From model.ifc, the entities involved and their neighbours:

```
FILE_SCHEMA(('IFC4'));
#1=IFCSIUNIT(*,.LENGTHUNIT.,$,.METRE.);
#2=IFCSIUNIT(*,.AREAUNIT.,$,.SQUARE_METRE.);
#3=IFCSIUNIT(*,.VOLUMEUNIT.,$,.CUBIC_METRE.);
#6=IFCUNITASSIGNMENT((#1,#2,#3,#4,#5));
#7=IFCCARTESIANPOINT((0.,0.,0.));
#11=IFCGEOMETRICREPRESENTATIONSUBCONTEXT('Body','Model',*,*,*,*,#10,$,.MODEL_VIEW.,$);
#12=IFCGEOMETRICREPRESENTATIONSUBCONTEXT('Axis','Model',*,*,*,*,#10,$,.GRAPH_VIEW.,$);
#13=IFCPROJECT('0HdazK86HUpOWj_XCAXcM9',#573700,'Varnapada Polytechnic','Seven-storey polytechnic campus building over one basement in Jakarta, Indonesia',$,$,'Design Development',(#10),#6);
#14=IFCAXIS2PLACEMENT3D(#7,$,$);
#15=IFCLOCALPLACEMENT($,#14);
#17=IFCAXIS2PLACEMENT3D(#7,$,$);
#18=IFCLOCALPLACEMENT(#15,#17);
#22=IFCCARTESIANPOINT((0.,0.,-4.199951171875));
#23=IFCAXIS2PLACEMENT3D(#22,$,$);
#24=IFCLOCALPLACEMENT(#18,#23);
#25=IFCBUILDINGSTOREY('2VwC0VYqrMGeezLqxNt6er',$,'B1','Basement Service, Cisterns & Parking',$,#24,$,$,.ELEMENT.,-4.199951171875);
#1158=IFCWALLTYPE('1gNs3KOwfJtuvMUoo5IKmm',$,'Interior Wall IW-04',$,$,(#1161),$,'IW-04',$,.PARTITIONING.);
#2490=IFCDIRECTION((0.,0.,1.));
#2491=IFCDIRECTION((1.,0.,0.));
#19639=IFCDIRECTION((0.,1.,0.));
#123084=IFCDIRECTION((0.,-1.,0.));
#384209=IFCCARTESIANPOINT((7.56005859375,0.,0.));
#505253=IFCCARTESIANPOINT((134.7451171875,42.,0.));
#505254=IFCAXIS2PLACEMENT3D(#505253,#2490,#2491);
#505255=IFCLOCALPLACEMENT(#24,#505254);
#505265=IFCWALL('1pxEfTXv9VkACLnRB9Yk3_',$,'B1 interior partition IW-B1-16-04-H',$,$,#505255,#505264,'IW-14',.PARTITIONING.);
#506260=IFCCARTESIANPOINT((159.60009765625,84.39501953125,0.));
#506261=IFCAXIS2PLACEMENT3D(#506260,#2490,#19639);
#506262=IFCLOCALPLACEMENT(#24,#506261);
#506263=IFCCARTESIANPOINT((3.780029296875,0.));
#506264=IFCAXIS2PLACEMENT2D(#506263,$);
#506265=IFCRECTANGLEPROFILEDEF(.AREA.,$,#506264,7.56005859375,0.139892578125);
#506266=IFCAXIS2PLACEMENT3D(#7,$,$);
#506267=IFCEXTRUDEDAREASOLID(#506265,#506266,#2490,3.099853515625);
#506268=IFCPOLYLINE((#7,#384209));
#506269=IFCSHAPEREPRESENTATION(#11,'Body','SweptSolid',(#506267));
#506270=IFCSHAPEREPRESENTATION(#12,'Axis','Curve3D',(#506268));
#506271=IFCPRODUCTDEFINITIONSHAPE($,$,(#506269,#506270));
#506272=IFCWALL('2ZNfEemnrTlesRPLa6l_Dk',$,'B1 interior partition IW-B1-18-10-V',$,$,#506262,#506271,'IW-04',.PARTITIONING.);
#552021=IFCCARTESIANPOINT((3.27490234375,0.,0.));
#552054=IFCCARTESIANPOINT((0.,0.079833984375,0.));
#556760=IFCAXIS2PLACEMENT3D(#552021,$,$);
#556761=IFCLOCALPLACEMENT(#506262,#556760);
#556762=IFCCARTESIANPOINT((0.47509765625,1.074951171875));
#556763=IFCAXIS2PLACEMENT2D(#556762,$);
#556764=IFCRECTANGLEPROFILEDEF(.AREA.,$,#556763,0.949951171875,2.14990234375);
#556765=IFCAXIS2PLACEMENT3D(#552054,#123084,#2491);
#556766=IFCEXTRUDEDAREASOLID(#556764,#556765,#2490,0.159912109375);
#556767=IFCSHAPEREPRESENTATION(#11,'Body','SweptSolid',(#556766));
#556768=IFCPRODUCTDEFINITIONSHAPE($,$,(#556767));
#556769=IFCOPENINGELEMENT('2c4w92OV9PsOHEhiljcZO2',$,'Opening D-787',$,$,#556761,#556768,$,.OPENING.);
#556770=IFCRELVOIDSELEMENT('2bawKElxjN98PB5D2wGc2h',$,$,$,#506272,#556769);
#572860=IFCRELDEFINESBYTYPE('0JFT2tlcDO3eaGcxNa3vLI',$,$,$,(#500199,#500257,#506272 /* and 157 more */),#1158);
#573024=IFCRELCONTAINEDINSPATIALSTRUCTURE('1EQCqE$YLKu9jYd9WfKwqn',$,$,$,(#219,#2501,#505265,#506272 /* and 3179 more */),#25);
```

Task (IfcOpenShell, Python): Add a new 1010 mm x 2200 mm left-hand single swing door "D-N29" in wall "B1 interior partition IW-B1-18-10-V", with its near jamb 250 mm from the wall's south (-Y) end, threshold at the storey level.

```python
import numpy as np
import ifcopenshell
import ifcopenshell.api.feature
import ifcopenshell.api.geometry
import ifcopenshell.api.root
import ifcopenshell.api.spatial
import ifcopenshell.geom
import ifcopenshell.util.element
import ifcopenshell.util.placement
import ifcopenshell.util.representation
import ifcopenshell.util.shape
import ifcopenshell.util.unit

model = ifcopenshell.open("model.ifc")
unit_scale = ifcopenshell.util.unit.calculate_unit_scale(model)
settings = ifcopenshell.geom.settings()


def volume(element):
    """Net volume in cubic metres, openings subtracted."""
    shape = ifcopenshell.geom.create_shape(settings, element)
    return ifcopenshell.util.shape.get_volume(shape.geometry)


wall = model.by_id(506272)
storey = ifcopenshell.util.element.get_container(wall, ifc_class="IfcBuildingStorey")
context = ifcopenshell.util.representation.get_context(model, "Model", "Body", "MODEL_VIEW")
before = volume(wall)

width, height, from_end, sill = 1.01, 2.2, 0.25, 0.0  # metres

# The wall runs along its own X axis, and the end named is its -X end.
wall_shape = ifcopenshell.geom.create_shape(settings, wall)
x, y, z = ifcopenshell.util.shape.get_vertices(wall_shape.geometry).T
start = x.min() + from_end
face, thickness = float(y.min()), float(y.max() - y.min())
wall_matrix = ifcopenshell.util.placement.get_local_placement(wall.ObjectPlacement)
level = ifcopenshell.util.placement.get_local_placement(storey.ObjectPlacement)[2, 3]


def in_wall(x, y):
    """Placement at x, y metres in the wall's axes, at sill height."""
    matrix = wall_matrix.copy()
    matrix[:, 3] = wall_matrix @ np.array([x / unit_scale, y / unit_scale, 0.0, 1.0])
    matrix[2, 3] = level + sill / unit_scale
    return matrix


# Opening: a box that overshoots both wall faces by 50 mm.
opening = ifcopenshell.api.root.create_entity(model, ifc_class="IfcOpeningElement", predefined_type="OPENING")
box = ifcopenshell.api.geometry.add_wall_representation(
    model, context=context, length=width, height=height, thickness=thickness + 0.1
)
ifcopenshell.api.geometry.assign_representation(model, product=opening, representation=box)
ifcopenshell.api.geometry.edit_object_placement(model, product=opening, matrix=in_wall(start, face - 0.05), is_si=False)
ifcopenshell.api.feature.add_feature(model, feature=opening, element=wall)

door = ifcopenshell.api.root.create_entity(model, ifc_class="IfcDoor", name="D-N29", predefined_type="DOOR")
door.OverallWidth, door.OverallHeight = width / unit_scale, height / unit_scale
door.OperationType = "SINGLE_SWING_LEFT"
body = ifcopenshell.api.geometry.add_door_representation(
    model,
    context=context,
    overall_width=door.OverallWidth,
    overall_height=door.OverallHeight,
    operation_type="SINGLE_SWING_LEFT",
    lining_properties={"LiningDepth": thickness / unit_scale, "ThresholdDepth": thickness / unit_scale},
)
ifcopenshell.api.geometry.assign_representation(model, product=door, representation=body)
ifcopenshell.api.spatial.assign_container(model, products=[door], relating_structure=storey)
ifcopenshell.api.feature.add_filling(model, opening=opening, element=door)

# The lining spans the wall, so the door starts at the wall face.
ifcopenshell.api.geometry.edit_object_placement(model, product=door, matrix=in_wall(start, face), is_si=False)

after = volume(wall)

print(f"wall volume {before:.3f} -> {after:.3f} m3")

model.write("model_edited.ifc")
```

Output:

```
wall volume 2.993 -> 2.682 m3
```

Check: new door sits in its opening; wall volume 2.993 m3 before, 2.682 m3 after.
